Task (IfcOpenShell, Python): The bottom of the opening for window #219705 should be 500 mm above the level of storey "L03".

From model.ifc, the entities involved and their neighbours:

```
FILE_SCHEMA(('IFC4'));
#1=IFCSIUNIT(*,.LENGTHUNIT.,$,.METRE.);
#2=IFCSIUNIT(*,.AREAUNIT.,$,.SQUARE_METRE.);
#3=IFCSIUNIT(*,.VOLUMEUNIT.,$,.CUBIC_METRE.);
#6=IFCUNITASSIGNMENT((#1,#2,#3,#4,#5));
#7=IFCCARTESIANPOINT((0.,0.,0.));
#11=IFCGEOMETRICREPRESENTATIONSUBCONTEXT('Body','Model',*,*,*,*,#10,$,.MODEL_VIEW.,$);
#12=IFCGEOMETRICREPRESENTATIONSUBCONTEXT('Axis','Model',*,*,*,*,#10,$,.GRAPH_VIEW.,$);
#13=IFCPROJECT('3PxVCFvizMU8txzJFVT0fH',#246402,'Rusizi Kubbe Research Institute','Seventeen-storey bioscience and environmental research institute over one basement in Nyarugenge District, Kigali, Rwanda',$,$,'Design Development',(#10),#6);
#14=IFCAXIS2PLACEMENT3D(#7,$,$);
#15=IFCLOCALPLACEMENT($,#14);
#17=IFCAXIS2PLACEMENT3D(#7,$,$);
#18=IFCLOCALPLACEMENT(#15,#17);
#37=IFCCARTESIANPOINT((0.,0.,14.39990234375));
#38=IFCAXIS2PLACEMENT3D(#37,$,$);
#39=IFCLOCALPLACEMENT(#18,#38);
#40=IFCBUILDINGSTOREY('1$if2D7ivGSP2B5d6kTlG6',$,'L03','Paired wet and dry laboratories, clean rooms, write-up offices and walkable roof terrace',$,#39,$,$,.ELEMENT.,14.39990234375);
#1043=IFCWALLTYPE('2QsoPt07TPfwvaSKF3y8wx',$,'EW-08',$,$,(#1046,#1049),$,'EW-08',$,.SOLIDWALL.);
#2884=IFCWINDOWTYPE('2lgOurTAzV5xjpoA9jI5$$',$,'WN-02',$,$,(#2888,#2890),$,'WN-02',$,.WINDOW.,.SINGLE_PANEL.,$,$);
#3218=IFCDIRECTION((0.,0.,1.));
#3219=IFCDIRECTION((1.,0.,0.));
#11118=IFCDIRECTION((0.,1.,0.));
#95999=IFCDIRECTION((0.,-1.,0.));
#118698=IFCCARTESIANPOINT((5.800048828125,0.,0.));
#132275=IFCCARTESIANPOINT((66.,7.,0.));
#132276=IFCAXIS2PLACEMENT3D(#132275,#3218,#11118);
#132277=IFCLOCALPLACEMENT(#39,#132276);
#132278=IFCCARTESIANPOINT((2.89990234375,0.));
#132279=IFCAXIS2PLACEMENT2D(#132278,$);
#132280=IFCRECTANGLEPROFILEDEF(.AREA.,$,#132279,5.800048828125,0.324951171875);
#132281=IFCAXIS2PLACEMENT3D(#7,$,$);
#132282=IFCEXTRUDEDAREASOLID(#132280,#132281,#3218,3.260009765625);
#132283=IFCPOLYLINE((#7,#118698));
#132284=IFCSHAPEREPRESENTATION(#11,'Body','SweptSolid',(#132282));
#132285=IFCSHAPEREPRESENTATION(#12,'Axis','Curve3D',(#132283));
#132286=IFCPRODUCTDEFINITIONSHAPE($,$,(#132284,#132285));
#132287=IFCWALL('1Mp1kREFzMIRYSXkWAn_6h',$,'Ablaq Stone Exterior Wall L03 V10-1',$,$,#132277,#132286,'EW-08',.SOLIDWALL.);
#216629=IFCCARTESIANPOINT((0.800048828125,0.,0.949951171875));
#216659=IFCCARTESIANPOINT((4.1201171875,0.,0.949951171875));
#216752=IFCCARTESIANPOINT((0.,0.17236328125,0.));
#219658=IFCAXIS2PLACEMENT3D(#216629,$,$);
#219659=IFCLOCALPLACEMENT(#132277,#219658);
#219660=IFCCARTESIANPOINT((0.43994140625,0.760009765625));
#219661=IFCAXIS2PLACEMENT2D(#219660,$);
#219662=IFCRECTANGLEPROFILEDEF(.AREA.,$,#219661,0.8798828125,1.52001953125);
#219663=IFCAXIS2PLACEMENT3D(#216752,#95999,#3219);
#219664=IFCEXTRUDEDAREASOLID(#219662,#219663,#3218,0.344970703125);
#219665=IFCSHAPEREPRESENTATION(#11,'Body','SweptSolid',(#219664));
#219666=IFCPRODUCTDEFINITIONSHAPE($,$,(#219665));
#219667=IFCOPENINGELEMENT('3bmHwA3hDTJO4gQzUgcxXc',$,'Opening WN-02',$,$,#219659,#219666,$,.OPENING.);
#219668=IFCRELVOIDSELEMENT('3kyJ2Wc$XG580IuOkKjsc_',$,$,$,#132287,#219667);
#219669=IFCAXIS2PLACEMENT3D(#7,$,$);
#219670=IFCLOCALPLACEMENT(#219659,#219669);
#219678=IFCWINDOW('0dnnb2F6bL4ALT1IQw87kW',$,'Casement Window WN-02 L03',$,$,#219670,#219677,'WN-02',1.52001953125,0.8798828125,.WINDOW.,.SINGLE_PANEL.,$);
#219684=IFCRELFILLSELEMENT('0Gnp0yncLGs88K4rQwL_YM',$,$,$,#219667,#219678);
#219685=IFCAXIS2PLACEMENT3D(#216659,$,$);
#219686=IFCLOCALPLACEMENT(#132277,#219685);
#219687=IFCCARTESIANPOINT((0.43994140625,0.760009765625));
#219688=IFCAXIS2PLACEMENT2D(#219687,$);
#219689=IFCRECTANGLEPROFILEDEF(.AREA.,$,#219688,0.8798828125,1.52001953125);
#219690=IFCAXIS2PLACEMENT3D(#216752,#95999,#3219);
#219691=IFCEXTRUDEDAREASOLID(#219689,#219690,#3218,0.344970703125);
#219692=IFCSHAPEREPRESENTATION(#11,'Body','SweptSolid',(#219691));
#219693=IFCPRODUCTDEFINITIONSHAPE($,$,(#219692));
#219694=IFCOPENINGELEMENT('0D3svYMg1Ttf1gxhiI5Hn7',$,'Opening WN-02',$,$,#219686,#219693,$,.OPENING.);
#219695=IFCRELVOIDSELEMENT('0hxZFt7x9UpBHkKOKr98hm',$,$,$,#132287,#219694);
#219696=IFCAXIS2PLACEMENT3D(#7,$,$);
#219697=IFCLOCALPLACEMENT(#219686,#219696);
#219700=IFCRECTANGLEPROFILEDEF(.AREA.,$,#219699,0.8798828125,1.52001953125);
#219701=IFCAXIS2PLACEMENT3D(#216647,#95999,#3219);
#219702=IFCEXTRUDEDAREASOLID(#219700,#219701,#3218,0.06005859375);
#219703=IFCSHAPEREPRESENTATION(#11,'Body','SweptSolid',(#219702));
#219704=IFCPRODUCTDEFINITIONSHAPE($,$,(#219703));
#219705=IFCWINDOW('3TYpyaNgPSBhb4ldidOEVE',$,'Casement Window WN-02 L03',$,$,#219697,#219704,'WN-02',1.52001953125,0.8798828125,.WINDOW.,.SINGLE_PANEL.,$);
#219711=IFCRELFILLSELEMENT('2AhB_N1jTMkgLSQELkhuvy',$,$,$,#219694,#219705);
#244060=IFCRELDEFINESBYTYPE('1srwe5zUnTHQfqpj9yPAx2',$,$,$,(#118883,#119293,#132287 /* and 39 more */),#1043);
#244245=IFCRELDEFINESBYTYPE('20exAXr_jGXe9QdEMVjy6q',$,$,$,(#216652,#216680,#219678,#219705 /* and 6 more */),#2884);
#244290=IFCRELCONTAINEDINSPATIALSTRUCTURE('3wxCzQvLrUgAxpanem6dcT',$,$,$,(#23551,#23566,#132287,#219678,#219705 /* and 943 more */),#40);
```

```python
import numpy as np
import ifcopenshell
import ifcopenshell.api.geometry
import ifcopenshell.geom
import ifcopenshell.util.element
import ifcopenshell.util.placement
import ifcopenshell.util.shape
import ifcopenshell.util.unit

model = ifcopenshell.open("model.ifc")
unit_scale = ifcopenshell.util.unit.calculate_unit_scale(model)

window = model.by_guid("3TYpyaNgPSBhb4ldidOEVE")
opening = window.FillsVoids[0].RelatingOpeningElement
storey = ifcopenshell.util.element.get_container(window, ifc_class="IfcBuildingStorey")
level = ifcopenshell.util.placement.get_local_placement(storey.ObjectPlacement)[2, 3]

# The opening's origin need not be at the sill, so measure its lowest point.
shape = ifcopenshell.geom.create_shape(ifcopenshell.geom.settings(), opening)
bottom = ifcopenshell.util.shape.get_shape_bottom_elevation(shape, shape.geometry) / unit_scale
dz = level + 0.5 / unit_scale - bottom

shift = np.array([0.0, 0.0, dz])
# The window is placed relative to its opening, so it follows when the opening moves.
matrix = ifcopenshell.util.placement.get_local_placement(opening.ObjectPlacement)
matrix[:3, 3] += shift
ifcopenshell.api.geometry.edit_object_placement(
    model, product=opening, matrix=matrix, is_si=False, should_transform_children=True
)

print(f"moved by {dz * unit_scale:+.3f} m")

model.write("model_v2.ifc")
```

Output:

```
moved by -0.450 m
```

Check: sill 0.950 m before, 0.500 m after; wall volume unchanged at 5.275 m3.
